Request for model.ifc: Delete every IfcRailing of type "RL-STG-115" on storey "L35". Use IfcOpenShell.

First a look at what the model holds.

```python
import ifcopenshell
import ifcopenshell.util.element

model = ifcopenshell.open("model.ifc")
print(model.schema)
storey = next(s for s in model.by_type("IfcBuildingStorey") if s.Name == "L35")
railings = [e for e in ifcopenshell.util.element.get_decomposition(storey) if e.is_a("IfcRailing")]
seen = {}
for e in railings:
    element_type = ifcopenshell.util.element.get_type(e)
    name = element_type.Name if element_type not in (None, e) else None
    seen[name] = seen.get(name, 0) + 1
for name, count in sorted(seen.items(), key=str):
    print(count, "x", name)
```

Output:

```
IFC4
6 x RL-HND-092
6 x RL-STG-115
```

```python
import ifcopenshell
import ifcopenshell.api.root
import ifcopenshell.util.element

model = ifcopenshell.open("model.ifc")

storey = next(s for s in model.by_type("IfcBuildingStorey") if s.Name == "L35")
railings = [e for e in ifcopenshell.util.element.get_decomposition(storey) if e.is_a("IfcRailing")]
targets = [e for e in railings if (t := ifcopenshell.util.element.get_type(e)) not in (None, e) and t.Name == "RL-STG-115"]

for e in targets:
    ifcopenshell.api.root.remove_product(model, product=e)
print(len(targets), "removed")

model.write("model_v2.ifc")
```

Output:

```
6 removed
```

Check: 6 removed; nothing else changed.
